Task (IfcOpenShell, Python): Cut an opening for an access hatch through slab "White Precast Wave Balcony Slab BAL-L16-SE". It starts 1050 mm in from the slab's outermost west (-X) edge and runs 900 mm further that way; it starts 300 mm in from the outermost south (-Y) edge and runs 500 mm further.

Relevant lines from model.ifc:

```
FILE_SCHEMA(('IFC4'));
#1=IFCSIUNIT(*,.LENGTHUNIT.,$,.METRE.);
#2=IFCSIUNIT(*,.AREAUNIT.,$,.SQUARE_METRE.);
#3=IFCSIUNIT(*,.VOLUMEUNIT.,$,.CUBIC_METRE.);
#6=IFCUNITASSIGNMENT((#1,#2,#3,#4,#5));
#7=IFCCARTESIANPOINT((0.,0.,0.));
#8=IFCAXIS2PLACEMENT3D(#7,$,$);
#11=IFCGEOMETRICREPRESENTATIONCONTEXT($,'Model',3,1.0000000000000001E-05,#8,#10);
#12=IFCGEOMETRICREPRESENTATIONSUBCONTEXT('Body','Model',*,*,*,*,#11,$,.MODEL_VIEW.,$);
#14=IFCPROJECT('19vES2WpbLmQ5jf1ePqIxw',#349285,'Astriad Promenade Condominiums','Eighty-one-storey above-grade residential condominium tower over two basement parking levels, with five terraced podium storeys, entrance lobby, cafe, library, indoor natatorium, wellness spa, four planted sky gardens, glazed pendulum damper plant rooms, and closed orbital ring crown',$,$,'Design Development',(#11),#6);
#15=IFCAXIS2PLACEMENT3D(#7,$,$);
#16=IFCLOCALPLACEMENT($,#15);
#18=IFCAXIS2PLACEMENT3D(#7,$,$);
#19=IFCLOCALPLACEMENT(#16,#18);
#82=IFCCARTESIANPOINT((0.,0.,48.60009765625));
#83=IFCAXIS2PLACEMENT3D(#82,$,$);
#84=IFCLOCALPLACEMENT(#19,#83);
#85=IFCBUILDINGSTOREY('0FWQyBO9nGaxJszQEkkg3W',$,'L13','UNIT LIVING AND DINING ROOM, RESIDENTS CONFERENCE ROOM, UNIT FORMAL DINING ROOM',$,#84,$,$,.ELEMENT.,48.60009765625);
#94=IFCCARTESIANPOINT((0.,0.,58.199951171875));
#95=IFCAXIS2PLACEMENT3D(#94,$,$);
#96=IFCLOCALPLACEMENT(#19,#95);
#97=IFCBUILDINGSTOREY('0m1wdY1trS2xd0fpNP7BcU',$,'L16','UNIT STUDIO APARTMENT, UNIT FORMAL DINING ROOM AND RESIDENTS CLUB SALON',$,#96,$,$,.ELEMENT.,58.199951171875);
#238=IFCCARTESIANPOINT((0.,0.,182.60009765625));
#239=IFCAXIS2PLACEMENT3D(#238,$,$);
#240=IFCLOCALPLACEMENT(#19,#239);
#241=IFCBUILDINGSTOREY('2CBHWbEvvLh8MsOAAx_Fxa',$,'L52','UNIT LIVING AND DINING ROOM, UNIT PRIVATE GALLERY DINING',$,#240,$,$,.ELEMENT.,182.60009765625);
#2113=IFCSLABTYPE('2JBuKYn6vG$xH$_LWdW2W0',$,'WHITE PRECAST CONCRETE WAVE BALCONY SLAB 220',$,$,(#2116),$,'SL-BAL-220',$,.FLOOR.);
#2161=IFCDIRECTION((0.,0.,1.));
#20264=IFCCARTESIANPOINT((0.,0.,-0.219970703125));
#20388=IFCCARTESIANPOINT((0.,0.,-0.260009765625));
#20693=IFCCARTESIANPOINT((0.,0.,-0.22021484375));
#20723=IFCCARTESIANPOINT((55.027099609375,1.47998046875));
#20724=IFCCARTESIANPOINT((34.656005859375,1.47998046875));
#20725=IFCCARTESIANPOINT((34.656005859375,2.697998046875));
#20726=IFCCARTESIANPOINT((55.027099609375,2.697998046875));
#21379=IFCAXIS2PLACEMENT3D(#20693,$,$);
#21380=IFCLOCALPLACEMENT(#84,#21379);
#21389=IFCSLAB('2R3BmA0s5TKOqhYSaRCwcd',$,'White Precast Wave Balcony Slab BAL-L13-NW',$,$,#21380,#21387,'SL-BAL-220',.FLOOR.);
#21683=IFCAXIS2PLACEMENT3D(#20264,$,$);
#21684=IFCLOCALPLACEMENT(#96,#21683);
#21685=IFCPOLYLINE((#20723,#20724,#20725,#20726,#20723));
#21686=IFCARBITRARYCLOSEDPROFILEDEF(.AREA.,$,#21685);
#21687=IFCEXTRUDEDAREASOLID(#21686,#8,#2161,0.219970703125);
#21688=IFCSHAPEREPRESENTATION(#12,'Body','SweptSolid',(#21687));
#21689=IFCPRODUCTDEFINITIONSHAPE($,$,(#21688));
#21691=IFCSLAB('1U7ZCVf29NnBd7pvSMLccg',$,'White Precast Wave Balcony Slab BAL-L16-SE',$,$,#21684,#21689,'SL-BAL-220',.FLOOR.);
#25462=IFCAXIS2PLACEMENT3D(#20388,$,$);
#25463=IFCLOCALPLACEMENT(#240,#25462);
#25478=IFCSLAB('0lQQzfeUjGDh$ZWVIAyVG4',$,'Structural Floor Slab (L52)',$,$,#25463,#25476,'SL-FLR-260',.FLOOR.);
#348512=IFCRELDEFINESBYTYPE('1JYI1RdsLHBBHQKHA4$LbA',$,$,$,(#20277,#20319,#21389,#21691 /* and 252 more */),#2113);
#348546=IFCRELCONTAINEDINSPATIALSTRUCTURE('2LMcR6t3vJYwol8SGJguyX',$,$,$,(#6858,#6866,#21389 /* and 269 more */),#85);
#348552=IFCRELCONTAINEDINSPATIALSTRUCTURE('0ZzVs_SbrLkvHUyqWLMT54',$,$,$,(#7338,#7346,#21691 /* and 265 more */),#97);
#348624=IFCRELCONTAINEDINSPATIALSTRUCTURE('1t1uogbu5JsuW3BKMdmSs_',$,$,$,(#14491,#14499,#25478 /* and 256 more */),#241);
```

```python
import numpy as np
import ifcopenshell
import ifcopenshell.api.feature
import ifcopenshell.api.geometry
import ifcopenshell.api.root
import ifcopenshell.geom
import ifcopenshell.util.placement
import ifcopenshell.util.representation
import ifcopenshell.util.shape
import ifcopenshell.util.unit

model = ifcopenshell.open("model.ifc")
unit_scale = ifcopenshell.util.unit.calculate_unit_scale(model)
settings = ifcopenshell.geom.settings()


def volume(element):
    """Net volume in cubic metres, openings subtracted."""
    shape = ifcopenshell.geom.create_shape(settings, element)
    return ifcopenshell.util.shape.get_volume(shape.geometry)


slab = model.by_guid("1U7ZCVf29NnBd7pvSMLccg")
before = volume(slab)

# Extent in the slab's own axes, in metres. The edges named are its -X and -Y sides.
slab_shape = ifcopenshell.geom.create_shape(settings, slab)
vertices = ifcopenshell.util.shape.get_vertices(slab_shape.geometry)
x_min, y_min, bottom = vertices.min(axis=0)
top = vertices[:, 2].max()

opening = ifcopenshell.api.root.create_entity(model, ifc_class="IfcOpeningElement", name="Access hatch opening", predefined_type="OPENING")
context = ifcopenshell.util.representation.get_context(model, "Model", "Body", "MODEL_VIEW")
width, depth = 0.9, 0.5
outline = [(0.0, 0.0), (width, 0.0), (width, depth), (0.0, depth), (0.0, 0.0)]
# Overshoot both faces by 50 mm so the cut is clean.
shape = ifcopenshell.api.geometry.add_slab_representation(
    model, context=context, depth=top - bottom + 0.1, polyline=outline
)
ifcopenshell.api.geometry.assign_representation(model, product=opening, representation=shape)

matrix = ifcopenshell.util.placement.get_local_placement(slab.ObjectPlacement)
matrix[:, 3] = matrix @ np.append(np.array([x_min + 1.05, y_min + 0.3, bottom - 0.05]) / unit_scale, 1.0)
ifcopenshell.api.geometry.edit_object_placement(model, product=opening, matrix=matrix, is_si=False)
ifcopenshell.api.feature.add_feature(model, feature=opening, element=slab)

after = volume(slab)

print(f"slab volume {before:.3f} -> {after:.3f} m3")

model.write("model_v2.ifc")
```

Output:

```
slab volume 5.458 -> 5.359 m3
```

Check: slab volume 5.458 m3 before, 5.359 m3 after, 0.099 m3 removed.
